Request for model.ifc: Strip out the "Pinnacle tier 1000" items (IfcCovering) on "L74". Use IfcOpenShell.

First a look at what the model holds.

```python
import ifcopenshell
import ifcopenshell.util.element

model = ifcopenshell.open("model.ifc")
print(model.schema)
storey = next(s for s in model.by_type("IfcBuildingStorey") if s.Name == "L74")
coverings = [e for e in ifcopenshell.util.element.get_decomposition(storey) if e.is_a("IfcCovering")]
seen = {}
for e in coverings:
    element_type = ifcopenshell.util.element.get_type(e)
    name = element_type.Name if element_type not in (None, e) else None
    seen[name] = seen.get(name, 0) + 1
for name, count in sorted(seen.items(), key=str):
    print(count, "x", name)
```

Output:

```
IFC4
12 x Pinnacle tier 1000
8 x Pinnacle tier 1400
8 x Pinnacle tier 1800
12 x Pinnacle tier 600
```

```python
import ifcopenshell
import ifcopenshell.api.root
import ifcopenshell.util.element

model = ifcopenshell.open("model.ifc")

storey = next(s for s in model.by_type("IfcBuildingStorey") if s.Name == "L74")
coverings = [e for e in ifcopenshell.util.element.get_decomposition(storey) if e.is_a("IfcCovering")]
targets = [e for e in coverings if (t := ifcopenshell.util.element.get_type(e)) not in (None, e) and t.Name == "Pinnacle tier 1000"]

for e in targets:
    ifcopenshell.api.root.remove_product(model, product=e)
print(len(targets), "removed")

model.write("model_v2.ifc")
```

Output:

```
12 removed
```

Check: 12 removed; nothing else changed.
